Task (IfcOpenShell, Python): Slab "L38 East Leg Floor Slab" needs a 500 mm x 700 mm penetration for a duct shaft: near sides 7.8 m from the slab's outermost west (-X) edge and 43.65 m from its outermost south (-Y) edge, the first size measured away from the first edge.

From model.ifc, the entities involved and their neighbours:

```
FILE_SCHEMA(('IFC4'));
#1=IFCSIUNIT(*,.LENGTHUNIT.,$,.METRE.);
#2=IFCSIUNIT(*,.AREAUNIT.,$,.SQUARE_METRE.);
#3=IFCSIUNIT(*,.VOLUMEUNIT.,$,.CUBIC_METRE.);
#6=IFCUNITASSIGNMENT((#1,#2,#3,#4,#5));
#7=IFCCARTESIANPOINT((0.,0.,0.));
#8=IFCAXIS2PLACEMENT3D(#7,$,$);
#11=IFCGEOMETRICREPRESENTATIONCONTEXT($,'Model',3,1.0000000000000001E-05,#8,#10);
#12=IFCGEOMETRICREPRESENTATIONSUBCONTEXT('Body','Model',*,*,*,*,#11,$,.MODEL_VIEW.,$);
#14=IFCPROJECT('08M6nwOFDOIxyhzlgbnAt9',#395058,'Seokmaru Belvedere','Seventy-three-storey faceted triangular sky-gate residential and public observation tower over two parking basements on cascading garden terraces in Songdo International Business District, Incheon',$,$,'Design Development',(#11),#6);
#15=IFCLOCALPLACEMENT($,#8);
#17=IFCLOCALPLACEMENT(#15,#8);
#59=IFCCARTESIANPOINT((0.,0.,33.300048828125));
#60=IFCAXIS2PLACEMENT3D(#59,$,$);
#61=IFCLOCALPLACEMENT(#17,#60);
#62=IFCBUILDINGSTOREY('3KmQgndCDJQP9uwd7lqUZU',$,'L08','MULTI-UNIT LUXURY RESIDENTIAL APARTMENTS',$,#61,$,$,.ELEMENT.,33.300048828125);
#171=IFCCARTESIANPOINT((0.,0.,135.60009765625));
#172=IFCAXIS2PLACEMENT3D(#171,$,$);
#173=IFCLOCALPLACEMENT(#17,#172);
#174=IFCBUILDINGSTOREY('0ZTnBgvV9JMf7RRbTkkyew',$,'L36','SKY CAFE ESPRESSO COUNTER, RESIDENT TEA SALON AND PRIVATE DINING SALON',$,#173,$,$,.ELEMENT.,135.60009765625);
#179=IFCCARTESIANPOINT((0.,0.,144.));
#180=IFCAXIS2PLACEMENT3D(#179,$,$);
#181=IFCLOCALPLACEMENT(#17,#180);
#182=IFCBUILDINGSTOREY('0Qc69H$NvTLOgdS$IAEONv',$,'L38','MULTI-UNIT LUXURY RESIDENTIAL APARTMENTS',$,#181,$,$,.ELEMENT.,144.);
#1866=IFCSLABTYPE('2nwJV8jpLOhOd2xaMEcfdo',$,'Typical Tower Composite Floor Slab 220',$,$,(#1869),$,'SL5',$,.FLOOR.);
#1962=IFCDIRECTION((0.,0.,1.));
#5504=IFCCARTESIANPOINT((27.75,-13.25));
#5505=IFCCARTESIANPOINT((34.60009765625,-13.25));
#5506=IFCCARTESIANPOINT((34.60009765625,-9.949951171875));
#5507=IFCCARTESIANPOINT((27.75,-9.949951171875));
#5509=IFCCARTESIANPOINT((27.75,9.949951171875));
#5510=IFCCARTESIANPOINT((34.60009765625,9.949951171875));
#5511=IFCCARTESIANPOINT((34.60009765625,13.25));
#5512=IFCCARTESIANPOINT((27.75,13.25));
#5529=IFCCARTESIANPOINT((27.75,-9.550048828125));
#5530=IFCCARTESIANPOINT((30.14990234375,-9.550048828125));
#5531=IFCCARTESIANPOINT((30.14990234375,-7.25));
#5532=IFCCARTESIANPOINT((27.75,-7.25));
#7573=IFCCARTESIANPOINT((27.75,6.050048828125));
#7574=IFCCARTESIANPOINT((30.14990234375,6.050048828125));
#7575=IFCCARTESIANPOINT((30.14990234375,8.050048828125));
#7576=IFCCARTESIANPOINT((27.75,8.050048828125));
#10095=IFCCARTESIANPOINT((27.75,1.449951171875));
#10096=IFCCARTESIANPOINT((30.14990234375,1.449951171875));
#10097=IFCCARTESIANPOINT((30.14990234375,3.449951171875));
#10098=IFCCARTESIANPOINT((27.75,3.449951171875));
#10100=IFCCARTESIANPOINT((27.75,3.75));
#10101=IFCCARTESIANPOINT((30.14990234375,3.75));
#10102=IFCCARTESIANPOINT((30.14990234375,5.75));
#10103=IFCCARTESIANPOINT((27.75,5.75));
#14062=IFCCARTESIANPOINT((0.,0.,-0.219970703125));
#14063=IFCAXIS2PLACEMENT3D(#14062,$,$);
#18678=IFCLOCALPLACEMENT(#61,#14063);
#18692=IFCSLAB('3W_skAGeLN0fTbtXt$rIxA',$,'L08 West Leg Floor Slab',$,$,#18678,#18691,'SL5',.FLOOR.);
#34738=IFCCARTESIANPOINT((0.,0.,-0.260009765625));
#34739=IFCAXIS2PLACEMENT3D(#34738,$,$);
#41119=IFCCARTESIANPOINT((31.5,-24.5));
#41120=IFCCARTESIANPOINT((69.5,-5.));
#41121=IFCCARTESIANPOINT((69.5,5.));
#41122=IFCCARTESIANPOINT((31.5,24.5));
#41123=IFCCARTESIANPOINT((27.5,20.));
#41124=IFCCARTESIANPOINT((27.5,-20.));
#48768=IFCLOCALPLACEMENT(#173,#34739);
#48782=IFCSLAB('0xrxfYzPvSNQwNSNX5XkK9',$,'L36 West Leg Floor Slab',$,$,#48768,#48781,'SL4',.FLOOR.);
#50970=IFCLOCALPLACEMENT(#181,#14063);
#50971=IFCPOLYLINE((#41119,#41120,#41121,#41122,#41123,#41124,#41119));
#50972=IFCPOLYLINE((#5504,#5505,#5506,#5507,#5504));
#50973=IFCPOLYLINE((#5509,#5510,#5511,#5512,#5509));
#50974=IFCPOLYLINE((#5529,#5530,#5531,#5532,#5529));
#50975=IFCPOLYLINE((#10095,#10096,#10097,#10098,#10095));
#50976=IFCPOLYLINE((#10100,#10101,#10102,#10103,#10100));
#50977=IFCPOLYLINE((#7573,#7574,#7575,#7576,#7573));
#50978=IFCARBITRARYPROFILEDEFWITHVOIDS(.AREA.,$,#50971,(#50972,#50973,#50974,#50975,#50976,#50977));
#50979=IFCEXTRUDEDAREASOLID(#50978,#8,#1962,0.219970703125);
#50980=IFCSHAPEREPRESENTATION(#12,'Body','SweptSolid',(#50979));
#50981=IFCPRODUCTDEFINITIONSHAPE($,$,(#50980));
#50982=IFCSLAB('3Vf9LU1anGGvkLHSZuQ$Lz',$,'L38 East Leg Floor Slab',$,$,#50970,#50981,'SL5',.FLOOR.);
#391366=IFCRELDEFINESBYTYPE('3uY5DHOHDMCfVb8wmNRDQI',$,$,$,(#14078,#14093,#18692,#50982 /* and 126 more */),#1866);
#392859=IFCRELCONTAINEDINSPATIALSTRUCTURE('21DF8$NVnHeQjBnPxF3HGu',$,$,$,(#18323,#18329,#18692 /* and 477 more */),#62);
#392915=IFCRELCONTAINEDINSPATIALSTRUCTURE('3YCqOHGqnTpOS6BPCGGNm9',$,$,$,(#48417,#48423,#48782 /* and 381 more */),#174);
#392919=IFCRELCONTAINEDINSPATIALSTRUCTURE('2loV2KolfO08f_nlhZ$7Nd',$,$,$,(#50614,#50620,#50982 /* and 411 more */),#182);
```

```python
import numpy as np
import ifcopenshell
import ifcopenshell.api.feature
import ifcopenshell.api.geometry
import ifcopenshell.api.root
import ifcopenshell.geom
import ifcopenshell.util.placement
import ifcopenshell.util.representation
import ifcopenshell.util.shape
import ifcopenshell.util.unit

model = ifcopenshell.open("model.ifc")
unit_scale = ifcopenshell.util.unit.calculate_unit_scale(model)
settings = ifcopenshell.geom.settings()


def volume(element):
    """Net volume in cubic metres, openings subtracted."""
    shape = ifcopenshell.geom.create_shape(settings, element)
    return ifcopenshell.util.shape.get_volume(shape.geometry)


slab = model.by_guid("3Vf9LU1anGGvkLHSZuQ$Lz")
before = volume(slab)

# Extent in the slab's own axes, in metres. The edges named are its -X and -Y sides.
slab_shape = ifcopenshell.geom.create_shape(settings, slab)
vertices = ifcopenshell.util.shape.get_vertices(slab_shape.geometry)
x_min, y_min, bottom = vertices.min(axis=0)
top = vertices[:, 2].max()

opening = ifcopenshell.api.root.create_entity(model, ifc_class="IfcOpeningElement", name="Duct shaft opening", predefined_type="OPENING")
context = ifcopenshell.util.representation.get_context(model, "Model", "Body", "MODEL_VIEW")
width, depth = 0.5, 0.7
outline = [(0.0, 0.0), (width, 0.0), (width, depth), (0.0, depth), (0.0, 0.0)]
# Overshoot both faces by 50 mm so the cut is clean.
shape = ifcopenshell.api.geometry.add_slab_representation(
    model, context=context, depth=top - bottom + 0.1, polyline=outline
)
ifcopenshell.api.geometry.assign_representation(model, product=opening, representation=shape)

matrix = ifcopenshell.util.placement.get_local_placement(slab.ObjectPlacement)
matrix[:, 3] = matrix @ np.append(np.array([x_min + 7.8, y_min + 43.65, bottom - 0.05]) / unit_scale, 1.0)
ifcopenshell.api.geometry.edit_object_placement(model, product=opening, matrix=matrix, is_si=False)
ifcopenshell.api.feature.add_feature(model, feature=opening, element=slab)

after = volume(slab)

print(f"slab volume {before:.3f} -> {after:.3f} m3")

model.write("model-out.ifc")
```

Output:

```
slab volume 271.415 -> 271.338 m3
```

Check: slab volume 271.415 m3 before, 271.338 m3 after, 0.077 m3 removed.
